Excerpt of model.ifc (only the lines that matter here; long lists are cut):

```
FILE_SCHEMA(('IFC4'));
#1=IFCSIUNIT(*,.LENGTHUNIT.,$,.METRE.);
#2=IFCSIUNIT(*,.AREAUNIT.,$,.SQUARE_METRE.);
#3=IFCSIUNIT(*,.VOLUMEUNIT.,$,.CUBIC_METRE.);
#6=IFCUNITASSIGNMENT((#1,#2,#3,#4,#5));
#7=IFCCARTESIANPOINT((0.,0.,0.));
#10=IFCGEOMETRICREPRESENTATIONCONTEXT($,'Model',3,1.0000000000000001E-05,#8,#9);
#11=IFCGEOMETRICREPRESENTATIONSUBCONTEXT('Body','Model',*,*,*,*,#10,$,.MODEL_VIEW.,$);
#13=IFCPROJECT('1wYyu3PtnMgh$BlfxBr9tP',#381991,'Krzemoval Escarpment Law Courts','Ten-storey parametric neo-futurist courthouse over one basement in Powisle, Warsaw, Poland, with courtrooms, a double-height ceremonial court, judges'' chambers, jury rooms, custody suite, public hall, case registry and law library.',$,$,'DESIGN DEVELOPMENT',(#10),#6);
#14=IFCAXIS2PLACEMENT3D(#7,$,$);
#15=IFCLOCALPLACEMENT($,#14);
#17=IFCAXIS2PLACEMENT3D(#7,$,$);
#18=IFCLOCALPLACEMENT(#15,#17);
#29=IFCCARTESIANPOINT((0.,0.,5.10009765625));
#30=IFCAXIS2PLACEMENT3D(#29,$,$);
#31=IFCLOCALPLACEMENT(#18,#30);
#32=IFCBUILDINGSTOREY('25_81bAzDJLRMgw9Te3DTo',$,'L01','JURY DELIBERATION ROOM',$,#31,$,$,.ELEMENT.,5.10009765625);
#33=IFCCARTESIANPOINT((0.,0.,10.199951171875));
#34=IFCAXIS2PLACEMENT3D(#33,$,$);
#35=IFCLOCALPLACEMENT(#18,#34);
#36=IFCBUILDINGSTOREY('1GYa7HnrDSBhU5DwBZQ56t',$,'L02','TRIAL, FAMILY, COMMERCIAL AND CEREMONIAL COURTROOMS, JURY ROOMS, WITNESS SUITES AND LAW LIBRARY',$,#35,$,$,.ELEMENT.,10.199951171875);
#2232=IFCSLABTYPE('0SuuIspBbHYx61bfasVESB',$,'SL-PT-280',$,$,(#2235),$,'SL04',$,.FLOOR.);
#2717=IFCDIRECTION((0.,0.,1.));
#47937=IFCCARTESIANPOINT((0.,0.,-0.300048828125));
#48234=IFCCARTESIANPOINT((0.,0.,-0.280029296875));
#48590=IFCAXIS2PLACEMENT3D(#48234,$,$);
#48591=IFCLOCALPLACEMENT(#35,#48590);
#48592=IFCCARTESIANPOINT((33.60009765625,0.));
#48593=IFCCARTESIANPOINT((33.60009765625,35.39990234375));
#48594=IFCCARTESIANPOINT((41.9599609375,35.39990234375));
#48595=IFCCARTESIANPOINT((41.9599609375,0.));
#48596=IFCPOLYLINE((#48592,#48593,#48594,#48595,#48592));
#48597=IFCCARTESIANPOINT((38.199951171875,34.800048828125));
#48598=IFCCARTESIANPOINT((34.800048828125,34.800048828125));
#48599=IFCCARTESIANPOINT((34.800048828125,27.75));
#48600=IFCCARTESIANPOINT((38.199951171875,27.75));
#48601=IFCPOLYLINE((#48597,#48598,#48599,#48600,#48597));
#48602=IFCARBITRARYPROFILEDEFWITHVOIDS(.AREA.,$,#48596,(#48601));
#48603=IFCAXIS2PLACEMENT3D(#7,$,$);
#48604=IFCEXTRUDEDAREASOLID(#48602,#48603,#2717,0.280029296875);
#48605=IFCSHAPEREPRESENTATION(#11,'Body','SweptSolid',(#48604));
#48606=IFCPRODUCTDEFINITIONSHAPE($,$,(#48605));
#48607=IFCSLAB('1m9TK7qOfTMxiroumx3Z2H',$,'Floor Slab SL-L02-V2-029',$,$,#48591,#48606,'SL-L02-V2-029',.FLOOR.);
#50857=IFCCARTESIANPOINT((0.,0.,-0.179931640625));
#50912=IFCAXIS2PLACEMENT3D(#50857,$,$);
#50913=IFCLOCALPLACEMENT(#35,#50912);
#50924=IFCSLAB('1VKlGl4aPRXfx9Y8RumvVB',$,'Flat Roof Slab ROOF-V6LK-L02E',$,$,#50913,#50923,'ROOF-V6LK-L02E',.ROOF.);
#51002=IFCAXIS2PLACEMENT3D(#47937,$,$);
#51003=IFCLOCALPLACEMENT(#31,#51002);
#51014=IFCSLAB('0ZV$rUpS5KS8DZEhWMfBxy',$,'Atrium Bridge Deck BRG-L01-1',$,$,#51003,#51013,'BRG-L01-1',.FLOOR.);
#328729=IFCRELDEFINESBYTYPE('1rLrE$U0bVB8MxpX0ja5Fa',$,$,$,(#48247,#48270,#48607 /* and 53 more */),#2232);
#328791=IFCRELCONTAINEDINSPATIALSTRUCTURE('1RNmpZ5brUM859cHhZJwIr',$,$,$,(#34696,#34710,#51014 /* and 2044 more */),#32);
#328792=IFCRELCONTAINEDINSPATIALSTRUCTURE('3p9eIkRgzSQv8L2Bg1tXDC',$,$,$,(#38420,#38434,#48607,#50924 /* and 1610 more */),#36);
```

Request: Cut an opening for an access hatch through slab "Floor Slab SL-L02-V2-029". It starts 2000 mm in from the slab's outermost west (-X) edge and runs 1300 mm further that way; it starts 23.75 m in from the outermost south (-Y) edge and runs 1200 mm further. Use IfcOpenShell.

```python
import numpy as np
import ifcopenshell
import ifcopenshell.api.feature
import ifcopenshell.api.geometry
import ifcopenshell.api.root
import ifcopenshell.geom
import ifcopenshell.util.placement
import ifcopenshell.util.representation
import ifcopenshell.util.shape
import ifcopenshell.util.unit

model = ifcopenshell.open("model.ifc")
unit_scale = ifcopenshell.util.unit.calculate_unit_scale(model)
settings = ifcopenshell.geom.settings()


def volume(element):
    """Net volume in cubic metres, openings subtracted."""
    shape = ifcopenshell.geom.create_shape(settings, element)
    return ifcopenshell.util.shape.get_volume(shape.geometry)


slab = model.by_guid("1m9TK7qOfTMxiroumx3Z2H")
before = volume(slab)

# Extent in the slab's own axes, in metres. The edges named are its -X and -Y sides.
slab_shape = ifcopenshell.geom.create_shape(settings, slab)
vertices = ifcopenshell.util.shape.get_vertices(slab_shape.geometry)
x_min, y_min, bottom = vertices.min(axis=0)
top = vertices[:, 2].max()

opening = ifcopenshell.api.root.create_entity(model, ifc_class="IfcOpeningElement", name="Access hatch opening", predefined_type="OPENING")
context = ifcopenshell.util.representation.get_context(model, "Model", "Body", "MODEL_VIEW")
width, depth = 1.3, 1.2
outline = [(0.0, 0.0), (width, 0.0), (width, depth), (0.0, depth), (0.0, 0.0)]
# Overshoot both faces by 50 mm so the cut is clean.
shape = ifcopenshell.api.geometry.add_slab_representation(
    model, context=context, depth=top - bottom + 0.1, polyline=outline
)
ifcopenshell.api.geometry.assign_representation(model, product=opening, representation=shape)

matrix = ifcopenshell.util.placement.get_local_placement(slab.ObjectPlacement)
matrix[:, 3] = matrix @ np.append(np.array([x_min + 2, y_min + 23.75, bottom - 0.05]) / unit_scale, 1.0)
ifcopenshell.api.geometry.edit_object_placement(model, product=opening, matrix=matrix, is_si=False)
ifcopenshell.api.feature.add_feature(model, feature=opening, element=slab)

after = volume(slab)

print(f"slab volume {before:.3f} -> {after:.3f} m3")

model.write("model_rev.ifc")
```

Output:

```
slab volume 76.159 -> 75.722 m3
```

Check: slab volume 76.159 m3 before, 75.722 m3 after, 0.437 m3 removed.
